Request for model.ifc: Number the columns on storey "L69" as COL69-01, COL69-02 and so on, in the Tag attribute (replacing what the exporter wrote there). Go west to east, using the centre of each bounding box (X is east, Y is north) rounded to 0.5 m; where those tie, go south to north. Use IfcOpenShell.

First a look at what the model holds.

```python
import ifcopenshell
import ifcopenshell.util.element
import ifcopenshell.util.placement

model = ifcopenshell.open("model.ifc")
print(model.schema)
storey = next(s for s in model.by_type("IfcBuildingStorey") if s.Name == "L69")
columns = [e for e in ifcopenshell.util.element.get_decomposition(storey) if e.is_a("IfcColumn")]
for e in sorted(columns, key=lambda e: e.id()):
    origin = ifcopenshell.util.placement.get_local_placement(e.ObjectPlacement)[:3, 3]
    print(e.id(), e.Tag, e.Name, origin.round(2) + 0.0, sep=" | ")
```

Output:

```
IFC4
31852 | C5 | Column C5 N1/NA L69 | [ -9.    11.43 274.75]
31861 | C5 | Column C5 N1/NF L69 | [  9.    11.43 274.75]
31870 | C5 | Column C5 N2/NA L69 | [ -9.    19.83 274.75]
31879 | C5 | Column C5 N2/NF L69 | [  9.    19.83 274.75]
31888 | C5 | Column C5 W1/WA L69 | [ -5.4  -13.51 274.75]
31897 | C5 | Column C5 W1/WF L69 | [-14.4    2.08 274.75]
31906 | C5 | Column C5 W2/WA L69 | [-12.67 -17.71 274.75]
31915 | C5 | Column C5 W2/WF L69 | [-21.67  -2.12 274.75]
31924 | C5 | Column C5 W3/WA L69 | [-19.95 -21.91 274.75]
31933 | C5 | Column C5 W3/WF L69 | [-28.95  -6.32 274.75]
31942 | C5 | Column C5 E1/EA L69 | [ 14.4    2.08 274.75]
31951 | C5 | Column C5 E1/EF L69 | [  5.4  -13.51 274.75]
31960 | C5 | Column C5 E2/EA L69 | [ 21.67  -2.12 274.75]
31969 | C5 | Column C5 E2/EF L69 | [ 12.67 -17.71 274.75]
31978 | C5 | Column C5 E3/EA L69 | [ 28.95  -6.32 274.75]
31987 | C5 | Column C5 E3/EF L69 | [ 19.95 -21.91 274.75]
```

```python
import ifcopenshell
import ifcopenshell.geom
import ifcopenshell.util.element
import ifcopenshell.util.shape

model = ifcopenshell.open("model.ifc")
settings = ifcopenshell.geom.settings()
settings.set("use-world-coords", True)


def centre(element):
    shape = ifcopenshell.geom.create_shape(settings, element)
    return ifcopenshell.util.shape.get_bbox_centroid(shape.geometry)


storey = next(s for s in model.by_type("IfcBuildingStorey") if s.Name == "L69")
columns = [e for e in ifcopenshell.util.element.get_decomposition(storey) if e.is_a("IfcColumn")]

# Insertion points can sit at a corner or the storey origin, so sort by the geometry (in metres).
centres = {e: centre(e) for e in columns}
columns.sort(key=lambda e: (round(centres[e][0] / 0.5), centres[e][1]))

for i, e in enumerate(columns, start=1):
    number = f"COL69-{i:02d}"
    e.Tag = number
    print(e.id(), number)

model.write("model_v2.ifc")
```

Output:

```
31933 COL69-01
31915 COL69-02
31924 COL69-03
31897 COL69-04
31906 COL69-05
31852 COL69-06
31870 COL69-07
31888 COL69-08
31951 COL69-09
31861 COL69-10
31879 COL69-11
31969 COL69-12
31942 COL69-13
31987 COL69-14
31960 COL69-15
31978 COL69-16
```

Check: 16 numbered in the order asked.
